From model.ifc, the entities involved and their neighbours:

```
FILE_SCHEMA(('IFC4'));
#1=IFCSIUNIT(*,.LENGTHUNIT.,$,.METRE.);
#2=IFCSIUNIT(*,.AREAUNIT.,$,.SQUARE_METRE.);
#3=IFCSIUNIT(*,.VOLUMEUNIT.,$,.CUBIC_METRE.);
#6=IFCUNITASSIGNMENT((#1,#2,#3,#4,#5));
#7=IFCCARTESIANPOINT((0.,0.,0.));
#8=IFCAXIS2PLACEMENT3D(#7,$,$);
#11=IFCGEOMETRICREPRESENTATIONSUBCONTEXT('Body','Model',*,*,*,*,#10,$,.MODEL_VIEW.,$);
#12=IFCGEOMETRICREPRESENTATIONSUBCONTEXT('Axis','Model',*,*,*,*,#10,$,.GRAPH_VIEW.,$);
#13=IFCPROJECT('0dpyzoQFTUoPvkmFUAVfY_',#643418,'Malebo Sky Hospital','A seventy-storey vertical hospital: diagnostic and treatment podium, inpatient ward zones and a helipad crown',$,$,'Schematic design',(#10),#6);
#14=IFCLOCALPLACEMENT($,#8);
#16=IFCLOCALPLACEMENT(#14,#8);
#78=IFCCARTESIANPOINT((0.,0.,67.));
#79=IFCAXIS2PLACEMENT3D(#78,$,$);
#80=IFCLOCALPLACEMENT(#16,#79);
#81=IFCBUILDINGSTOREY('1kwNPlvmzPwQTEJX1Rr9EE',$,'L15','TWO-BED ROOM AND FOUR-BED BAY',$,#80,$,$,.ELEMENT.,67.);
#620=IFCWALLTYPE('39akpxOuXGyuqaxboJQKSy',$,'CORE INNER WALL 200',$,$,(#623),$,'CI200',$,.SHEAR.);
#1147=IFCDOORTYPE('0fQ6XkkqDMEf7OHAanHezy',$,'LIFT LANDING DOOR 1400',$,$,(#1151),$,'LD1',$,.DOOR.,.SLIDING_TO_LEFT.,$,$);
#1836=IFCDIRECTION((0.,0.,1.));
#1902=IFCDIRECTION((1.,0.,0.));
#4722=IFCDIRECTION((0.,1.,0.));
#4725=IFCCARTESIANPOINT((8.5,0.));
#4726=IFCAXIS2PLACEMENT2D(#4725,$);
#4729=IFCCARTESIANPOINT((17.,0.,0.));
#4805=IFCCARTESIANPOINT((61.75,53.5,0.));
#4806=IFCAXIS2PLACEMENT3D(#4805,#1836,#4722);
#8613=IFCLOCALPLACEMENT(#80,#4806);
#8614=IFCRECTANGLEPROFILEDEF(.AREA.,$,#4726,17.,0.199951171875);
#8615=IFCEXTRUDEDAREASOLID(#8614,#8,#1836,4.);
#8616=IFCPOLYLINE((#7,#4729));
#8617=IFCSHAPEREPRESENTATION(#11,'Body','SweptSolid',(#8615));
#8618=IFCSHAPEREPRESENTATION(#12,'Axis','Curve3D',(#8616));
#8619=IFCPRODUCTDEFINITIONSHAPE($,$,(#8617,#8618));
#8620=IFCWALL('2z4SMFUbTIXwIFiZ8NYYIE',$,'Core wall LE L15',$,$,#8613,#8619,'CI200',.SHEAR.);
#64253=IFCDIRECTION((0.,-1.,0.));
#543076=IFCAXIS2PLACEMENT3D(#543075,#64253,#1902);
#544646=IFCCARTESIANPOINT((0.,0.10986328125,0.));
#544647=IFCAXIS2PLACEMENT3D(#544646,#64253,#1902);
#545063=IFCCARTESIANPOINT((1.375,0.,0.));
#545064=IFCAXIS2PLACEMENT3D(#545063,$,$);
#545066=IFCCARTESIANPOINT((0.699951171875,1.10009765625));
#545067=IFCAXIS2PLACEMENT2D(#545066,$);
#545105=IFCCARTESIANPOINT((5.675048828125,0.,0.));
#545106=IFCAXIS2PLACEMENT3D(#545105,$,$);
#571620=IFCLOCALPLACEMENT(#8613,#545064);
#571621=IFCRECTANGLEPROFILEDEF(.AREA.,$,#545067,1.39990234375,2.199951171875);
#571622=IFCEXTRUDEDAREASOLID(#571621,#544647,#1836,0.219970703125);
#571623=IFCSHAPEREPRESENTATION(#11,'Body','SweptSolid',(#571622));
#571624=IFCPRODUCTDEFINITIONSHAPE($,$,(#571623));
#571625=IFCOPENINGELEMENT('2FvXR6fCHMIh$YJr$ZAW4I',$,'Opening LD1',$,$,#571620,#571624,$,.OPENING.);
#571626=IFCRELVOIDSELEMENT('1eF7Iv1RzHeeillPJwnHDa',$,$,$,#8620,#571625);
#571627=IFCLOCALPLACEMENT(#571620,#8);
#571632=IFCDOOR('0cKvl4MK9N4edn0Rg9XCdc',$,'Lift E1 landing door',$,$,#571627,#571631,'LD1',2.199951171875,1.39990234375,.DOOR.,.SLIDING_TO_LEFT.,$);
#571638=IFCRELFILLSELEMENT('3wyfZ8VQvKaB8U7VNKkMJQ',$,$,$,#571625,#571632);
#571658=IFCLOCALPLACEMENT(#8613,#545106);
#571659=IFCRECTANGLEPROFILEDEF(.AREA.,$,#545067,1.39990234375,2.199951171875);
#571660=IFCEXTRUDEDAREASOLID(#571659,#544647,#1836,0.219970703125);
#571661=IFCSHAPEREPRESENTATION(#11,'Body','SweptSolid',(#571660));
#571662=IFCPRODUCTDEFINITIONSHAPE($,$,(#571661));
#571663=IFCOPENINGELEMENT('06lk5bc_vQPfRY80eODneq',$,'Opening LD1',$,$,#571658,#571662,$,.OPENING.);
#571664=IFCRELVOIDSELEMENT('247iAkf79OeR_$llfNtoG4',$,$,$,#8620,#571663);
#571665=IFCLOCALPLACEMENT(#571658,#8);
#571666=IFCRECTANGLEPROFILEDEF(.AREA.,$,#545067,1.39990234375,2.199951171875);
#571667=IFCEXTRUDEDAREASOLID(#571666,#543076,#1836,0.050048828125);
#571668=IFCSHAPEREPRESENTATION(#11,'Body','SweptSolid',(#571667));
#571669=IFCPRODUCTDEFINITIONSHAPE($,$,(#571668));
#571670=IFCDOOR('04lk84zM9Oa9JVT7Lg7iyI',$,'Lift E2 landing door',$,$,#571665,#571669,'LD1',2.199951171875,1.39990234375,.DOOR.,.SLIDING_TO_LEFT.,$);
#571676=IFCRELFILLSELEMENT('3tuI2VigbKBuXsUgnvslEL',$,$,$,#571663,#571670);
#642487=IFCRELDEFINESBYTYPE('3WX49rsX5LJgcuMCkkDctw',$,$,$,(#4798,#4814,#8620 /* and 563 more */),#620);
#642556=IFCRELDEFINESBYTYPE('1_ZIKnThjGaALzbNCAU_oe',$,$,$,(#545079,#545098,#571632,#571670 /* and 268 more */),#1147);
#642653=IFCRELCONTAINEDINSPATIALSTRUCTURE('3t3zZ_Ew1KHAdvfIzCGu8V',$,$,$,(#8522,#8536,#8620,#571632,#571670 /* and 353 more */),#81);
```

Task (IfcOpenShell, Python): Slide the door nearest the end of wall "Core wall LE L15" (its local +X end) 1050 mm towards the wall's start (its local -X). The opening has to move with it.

```python
import ifcopenshell
import ifcopenshell.api.geometry
import ifcopenshell.util.placement
import ifcopenshell.util.unit

model = ifcopenshell.open("model.ifc")
unit_scale = ifcopenshell.util.unit.calculate_unit_scale(model)

door = model.by_guid("04lk84zM9Oa9JVT7Lg7iyI")
opening = door.FillsVoids[0].RelatingOpeningElement
wall = opening.VoidsElements[0].RelatingBuildingElement

wall_matrix = ifcopenshell.util.placement.get_local_placement(wall.ObjectPlacement)
shift = wall_matrix[:3, 0] * -1.05 / unit_scale
before = ifcopenshell.util.placement.get_local_placement(door.ObjectPlacement)[:3, 3].copy()

# The door is placed relative to its opening, so it follows when the opening moves.
matrix = ifcopenshell.util.placement.get_local_placement(opening.ObjectPlacement)
matrix[:3, 3] += shift
ifcopenshell.api.geometry.edit_object_placement(
    model, product=opening, matrix=matrix, is_si=False, should_transform_children=True
)

after = ifcopenshell.util.placement.get_local_placement(door.ObjectPlacement)[:3, 3]
print("door moved by", (after - before).round(3) + 0.0)

model.write("model_updated.ifc")
```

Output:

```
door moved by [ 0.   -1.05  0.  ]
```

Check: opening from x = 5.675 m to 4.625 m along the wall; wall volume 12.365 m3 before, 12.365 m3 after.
